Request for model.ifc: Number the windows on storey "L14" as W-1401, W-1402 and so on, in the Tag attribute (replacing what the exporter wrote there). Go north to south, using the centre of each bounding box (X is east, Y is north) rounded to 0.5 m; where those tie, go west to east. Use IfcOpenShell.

First a look at what the model holds.

```python
import ifcopenshell
import ifcopenshell.util.element
import ifcopenshell.util.placement

model = ifcopenshell.open("model.ifc")
print(model.schema)
storey = next(s for s in model.by_type("IfcBuildingStorey") if s.Name == "L14")
windows = [e for e in ifcopenshell.util.element.get_decomposition(storey) if e.is_a("IfcWindow")]
for e in sorted(windows, key=lambda e: e.id()):
    origin = ifcopenshell.util.placement.get_local_placement(e.ObjectPlacement)[:3, 3]
    print(e.id(), e.Tag, e.Name, origin.round(2) + 0.0, sep=" | ")
```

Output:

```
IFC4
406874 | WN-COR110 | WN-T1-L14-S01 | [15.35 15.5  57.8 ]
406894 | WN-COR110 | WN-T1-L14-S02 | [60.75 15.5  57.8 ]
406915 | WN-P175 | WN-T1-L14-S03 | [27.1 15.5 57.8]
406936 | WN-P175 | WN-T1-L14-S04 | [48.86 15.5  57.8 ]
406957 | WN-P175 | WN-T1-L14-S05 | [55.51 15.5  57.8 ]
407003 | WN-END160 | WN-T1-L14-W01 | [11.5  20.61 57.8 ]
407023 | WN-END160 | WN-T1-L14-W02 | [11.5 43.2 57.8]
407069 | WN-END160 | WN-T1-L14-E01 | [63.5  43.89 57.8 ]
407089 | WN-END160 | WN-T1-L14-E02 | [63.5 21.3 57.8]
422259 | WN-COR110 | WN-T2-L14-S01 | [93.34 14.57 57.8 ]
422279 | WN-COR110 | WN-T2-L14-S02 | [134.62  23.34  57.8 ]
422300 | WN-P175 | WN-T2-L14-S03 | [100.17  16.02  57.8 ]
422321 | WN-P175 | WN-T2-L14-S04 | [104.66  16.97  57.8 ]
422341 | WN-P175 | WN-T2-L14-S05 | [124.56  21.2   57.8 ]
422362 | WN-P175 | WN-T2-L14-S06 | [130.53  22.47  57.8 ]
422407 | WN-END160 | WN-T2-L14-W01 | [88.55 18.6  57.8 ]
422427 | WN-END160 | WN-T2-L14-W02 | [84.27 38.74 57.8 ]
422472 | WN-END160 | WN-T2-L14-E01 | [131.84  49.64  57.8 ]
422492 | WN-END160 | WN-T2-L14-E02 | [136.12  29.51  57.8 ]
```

```python
import ifcopenshell
import ifcopenshell.geom
import ifcopenshell.util.element
import ifcopenshell.util.shape

model = ifcopenshell.open("model.ifc")
settings = ifcopenshell.geom.settings()
settings.set("use-world-coords", True)


def centre(element):
    shape = ifcopenshell.geom.create_shape(settings, element)
    return ifcopenshell.util.shape.get_bbox_centroid(shape.geometry)


storey = next(s for s in model.by_type("IfcBuildingStorey") if s.Name == "L14")
windows = [e for e in ifcopenshell.util.element.get_decomposition(storey) if e.is_a("IfcWindow")]

# Insertion points can sit at a corner or the storey origin, so sort by the geometry (in metres).
centres = {e: centre(e) for e in windows}
windows.sort(key=lambda e: (-round(centres[e][1] / 0.5), centres[e][0]))

for i, e in enumerate(windows, start=1):
    number = f"W-14{i:02d}"
    e.Tag = number
    print(e.id(), number)

model.write("model_rev.ifc")
```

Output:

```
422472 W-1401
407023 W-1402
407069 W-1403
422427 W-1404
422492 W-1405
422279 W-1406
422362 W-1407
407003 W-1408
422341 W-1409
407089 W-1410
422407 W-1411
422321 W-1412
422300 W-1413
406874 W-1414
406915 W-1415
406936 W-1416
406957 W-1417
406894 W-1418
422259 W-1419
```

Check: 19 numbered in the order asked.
